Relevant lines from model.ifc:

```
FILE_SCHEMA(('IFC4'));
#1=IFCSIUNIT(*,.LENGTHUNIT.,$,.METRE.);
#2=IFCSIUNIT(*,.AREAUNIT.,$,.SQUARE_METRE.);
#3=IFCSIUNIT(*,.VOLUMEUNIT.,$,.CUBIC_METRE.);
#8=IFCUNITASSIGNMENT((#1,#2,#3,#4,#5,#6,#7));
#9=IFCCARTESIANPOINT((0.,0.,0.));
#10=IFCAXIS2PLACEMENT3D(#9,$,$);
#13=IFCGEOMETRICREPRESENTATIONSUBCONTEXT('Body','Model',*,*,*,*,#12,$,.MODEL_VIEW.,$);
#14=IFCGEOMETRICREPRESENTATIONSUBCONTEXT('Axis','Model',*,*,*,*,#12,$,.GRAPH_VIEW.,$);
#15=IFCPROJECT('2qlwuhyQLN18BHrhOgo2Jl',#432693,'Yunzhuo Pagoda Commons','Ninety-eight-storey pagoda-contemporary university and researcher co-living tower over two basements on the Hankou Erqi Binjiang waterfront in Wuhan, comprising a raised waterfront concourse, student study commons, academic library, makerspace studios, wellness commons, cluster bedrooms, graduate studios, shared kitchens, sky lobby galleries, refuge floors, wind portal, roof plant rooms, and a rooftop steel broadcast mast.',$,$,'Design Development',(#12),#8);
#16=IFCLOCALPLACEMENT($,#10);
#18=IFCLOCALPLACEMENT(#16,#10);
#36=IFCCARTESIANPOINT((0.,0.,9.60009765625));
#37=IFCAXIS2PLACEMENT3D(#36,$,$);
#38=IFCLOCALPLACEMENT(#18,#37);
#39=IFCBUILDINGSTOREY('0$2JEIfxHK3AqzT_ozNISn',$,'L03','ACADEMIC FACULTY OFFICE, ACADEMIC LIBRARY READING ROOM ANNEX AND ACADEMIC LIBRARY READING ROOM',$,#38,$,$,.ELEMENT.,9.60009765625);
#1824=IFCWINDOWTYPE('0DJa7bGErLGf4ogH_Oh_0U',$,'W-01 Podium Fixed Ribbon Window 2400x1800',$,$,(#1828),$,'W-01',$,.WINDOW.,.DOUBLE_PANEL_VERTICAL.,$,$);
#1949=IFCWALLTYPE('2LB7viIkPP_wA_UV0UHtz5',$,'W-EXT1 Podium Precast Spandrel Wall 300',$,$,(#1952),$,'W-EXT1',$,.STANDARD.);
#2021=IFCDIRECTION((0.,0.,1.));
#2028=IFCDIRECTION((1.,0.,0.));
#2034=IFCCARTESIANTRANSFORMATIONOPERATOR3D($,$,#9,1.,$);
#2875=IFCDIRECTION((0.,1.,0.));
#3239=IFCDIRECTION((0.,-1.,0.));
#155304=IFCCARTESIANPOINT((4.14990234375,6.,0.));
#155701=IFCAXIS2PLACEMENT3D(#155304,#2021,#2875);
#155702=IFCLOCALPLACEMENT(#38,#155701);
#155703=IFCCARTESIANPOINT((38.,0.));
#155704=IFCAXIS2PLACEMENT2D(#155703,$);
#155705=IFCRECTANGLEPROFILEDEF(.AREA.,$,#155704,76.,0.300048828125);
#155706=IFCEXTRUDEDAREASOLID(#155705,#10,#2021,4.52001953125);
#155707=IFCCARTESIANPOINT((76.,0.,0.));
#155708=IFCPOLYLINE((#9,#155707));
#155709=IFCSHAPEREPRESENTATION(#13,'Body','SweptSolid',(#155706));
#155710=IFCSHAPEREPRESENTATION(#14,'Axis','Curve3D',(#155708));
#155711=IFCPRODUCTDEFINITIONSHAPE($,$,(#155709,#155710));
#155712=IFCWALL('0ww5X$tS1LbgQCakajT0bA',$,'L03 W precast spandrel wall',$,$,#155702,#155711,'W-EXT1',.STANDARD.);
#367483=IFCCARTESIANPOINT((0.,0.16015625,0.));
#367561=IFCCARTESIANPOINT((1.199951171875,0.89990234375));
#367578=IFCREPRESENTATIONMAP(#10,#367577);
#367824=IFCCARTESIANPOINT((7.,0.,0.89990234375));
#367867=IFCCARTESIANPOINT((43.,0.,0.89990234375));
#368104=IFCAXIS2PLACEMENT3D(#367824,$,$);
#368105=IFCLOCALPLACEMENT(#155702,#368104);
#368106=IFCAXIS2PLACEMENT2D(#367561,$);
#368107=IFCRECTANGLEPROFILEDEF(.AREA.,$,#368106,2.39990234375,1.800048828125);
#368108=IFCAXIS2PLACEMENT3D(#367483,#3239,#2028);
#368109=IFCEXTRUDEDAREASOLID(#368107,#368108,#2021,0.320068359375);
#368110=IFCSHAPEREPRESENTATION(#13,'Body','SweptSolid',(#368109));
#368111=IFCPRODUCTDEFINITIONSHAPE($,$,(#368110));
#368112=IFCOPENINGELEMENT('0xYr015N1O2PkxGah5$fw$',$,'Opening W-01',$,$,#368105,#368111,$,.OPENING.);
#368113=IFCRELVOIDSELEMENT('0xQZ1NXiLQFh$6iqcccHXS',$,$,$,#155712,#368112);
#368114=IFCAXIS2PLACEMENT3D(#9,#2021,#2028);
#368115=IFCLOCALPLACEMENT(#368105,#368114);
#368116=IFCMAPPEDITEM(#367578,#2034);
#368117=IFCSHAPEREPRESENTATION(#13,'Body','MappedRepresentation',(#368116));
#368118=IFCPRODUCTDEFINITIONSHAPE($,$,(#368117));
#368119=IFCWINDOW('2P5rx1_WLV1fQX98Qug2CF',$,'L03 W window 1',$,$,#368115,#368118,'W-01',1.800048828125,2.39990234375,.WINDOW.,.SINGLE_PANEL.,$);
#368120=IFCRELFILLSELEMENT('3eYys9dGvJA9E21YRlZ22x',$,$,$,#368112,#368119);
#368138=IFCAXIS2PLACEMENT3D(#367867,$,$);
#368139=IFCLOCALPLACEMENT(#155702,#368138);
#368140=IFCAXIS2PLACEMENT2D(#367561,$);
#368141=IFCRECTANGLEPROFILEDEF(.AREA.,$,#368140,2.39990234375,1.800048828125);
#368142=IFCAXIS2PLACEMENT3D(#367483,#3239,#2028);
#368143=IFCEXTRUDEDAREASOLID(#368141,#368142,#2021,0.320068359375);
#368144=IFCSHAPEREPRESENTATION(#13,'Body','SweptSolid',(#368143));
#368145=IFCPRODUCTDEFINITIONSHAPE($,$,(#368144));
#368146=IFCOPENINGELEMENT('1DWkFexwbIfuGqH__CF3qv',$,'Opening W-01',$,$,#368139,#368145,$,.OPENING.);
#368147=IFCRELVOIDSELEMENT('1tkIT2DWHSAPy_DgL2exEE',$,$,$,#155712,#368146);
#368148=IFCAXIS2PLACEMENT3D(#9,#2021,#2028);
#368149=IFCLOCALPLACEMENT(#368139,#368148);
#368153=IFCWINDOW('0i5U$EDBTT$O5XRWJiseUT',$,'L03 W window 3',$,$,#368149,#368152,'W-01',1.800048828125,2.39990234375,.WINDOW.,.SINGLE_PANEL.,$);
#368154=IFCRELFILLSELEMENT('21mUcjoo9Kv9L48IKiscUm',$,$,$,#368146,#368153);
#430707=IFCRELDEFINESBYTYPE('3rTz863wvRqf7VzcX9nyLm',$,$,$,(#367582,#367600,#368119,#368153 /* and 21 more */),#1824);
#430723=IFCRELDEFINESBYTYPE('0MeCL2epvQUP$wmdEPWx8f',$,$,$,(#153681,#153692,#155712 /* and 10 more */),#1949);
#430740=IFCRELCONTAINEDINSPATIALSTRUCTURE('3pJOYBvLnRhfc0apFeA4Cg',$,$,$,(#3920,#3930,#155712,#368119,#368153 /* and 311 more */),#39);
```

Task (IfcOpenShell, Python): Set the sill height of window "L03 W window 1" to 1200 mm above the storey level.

```python
import numpy as np
import ifcopenshell
import ifcopenshell.api.geometry
import ifcopenshell.geom
import ifcopenshell.util.element
import ifcopenshell.util.placement
import ifcopenshell.util.shape
import ifcopenshell.util.unit

model = ifcopenshell.open("model.ifc")
unit_scale = ifcopenshell.util.unit.calculate_unit_scale(model)

window = model.by_guid("2P5rx1_WLV1fQX98Qug2CF")
opening = window.FillsVoids[0].RelatingOpeningElement
storey = ifcopenshell.util.element.get_container(window, ifc_class="IfcBuildingStorey")
level = ifcopenshell.util.placement.get_local_placement(storey.ObjectPlacement)[2, 3]

# The opening's origin need not be at the sill, so measure its lowest point.
shape = ifcopenshell.geom.create_shape(ifcopenshell.geom.settings(), opening)
bottom = ifcopenshell.util.shape.get_shape_bottom_elevation(shape, shape.geometry) / unit_scale
dz = level + 1.2 / unit_scale - bottom

shift = np.array([0.0, 0.0, dz])
# The window is placed relative to its opening, so it follows when the opening moves.
matrix = ifcopenshell.util.placement.get_local_placement(opening.ObjectPlacement)
matrix[:3, 3] += shift
ifcopenshell.api.geometry.edit_object_placement(
    model, product=opening, matrix=matrix, is_si=False, should_transform_children=True
)

print(f"moved by {dz * unit_scale:+.3f} m")

model.write("model_edited.ifc")
```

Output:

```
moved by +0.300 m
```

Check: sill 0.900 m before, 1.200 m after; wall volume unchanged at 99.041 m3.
